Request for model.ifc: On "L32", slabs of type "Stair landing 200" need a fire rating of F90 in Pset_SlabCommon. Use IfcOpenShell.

First a look at what the model holds.

```python
import ifcopenshell
import ifcopenshell.util.element

model = ifcopenshell.open("model.ifc")
print(model.schema)
storey = next(s for s in model.by_type("IfcBuildingStorey") if s.Name == "L32")
slabs = [e for e in ifcopenshell.util.element.get_decomposition(storey) if e.is_a("IfcSlab")]
seen = {}
for e in slabs:
    element_type = ifcopenshell.util.element.get_type(e)
    key = (element_type.Name if element_type != e and element_type else None, ifcopenshell.util.element.get_pset(e, "Pset_SlabCommon", "FireRating"))
    seen[key] = seen.get(key, 0) + 1
for (name, value), count in sorted(seen.items(), key=str):
    print(count, "x", name, "|", value)
```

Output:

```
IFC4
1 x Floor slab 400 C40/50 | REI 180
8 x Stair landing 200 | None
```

```python
import ifcopenshell
import ifcopenshell.api.pset
import ifcopenshell.util.element

model = ifcopenshell.open("model.ifc")

storey = next(s for s in model.by_type("IfcBuildingStorey") if s.Name == "L32")
slabs = [e for e in ifcopenshell.util.element.get_decomposition(storey) if e.is_a("IfcSlab")]

count = 0
for e in slabs:
    element_type = ifcopenshell.util.element.get_type(e)
    if element_type in (None, e) or element_type.Name != "Stair landing 200":
        continue
    found = ifcopenshell.util.element.get_pset(e, "Pset_SlabCommon", should_inherit=False)
    if found:
        pset = model.by_id(found["id"])
        if len(ifcopenshell.util.element.get_elements_by_pset(pset)) > 1:
            pset = ifcopenshell.api.pset.unshare_pset(model, products=[e], pset=pset)[0]
    else:
        pset = ifcopenshell.api.pset.add_pset(model, product=e, name="Pset_SlabCommon")
    ifcopenshell.api.pset.edit_pset(model, pset=pset, properties={"FireRating": "F90"})
    count += 1

print(count, "slabs updated")

model.write("model_rev.ifc")
```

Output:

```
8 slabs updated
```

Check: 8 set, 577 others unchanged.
